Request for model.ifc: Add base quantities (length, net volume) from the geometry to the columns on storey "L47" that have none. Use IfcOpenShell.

First a look at what the model holds.

```python
import ifcopenshell
import ifcopenshell.util.element
import ifcopenshell.util.unit

model = ifcopenshell.open("model.ifc")
print(model.schema)
for unit_type in ("LENGTHUNIT", "AREAUNIT", "VOLUMEUNIT"):
    print(unit_type, ifcopenshell.util.unit.calculate_unit_scale(model, unit_type))
storey = next(s for s in model.by_type("IfcBuildingStorey") if s.Name == "L47")
columns = [e for e in ifcopenshell.util.element.get_decomposition(storey) if e.is_a("IfcColumn")]
for e in sorted(columns, key=lambda e: e.id()):
    print(e.id(), e.is_a(), e.Name, list(ifcopenshell.util.element.get_psets(e, qtos_only=True)), sep=" | ")
```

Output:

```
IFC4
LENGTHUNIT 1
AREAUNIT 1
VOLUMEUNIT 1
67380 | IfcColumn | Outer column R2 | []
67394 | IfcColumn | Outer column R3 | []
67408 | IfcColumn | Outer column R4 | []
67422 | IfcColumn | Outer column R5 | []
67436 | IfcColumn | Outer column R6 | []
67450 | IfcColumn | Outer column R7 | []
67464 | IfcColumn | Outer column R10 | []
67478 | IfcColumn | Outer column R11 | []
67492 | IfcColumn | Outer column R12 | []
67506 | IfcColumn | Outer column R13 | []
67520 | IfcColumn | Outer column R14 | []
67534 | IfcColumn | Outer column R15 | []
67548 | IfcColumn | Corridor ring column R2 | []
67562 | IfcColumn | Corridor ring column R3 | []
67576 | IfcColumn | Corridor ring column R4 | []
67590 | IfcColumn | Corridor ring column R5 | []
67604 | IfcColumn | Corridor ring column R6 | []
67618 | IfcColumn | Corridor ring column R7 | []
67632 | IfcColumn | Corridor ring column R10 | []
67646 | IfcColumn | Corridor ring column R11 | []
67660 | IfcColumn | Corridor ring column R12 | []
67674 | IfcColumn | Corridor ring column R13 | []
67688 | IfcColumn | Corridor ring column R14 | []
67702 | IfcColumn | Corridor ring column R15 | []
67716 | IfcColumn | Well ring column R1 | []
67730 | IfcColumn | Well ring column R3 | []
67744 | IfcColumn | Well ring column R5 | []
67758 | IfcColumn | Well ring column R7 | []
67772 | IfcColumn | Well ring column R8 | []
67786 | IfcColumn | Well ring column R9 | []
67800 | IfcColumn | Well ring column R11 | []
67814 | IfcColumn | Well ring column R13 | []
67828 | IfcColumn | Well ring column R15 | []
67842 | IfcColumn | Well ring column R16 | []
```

```python
import ifcopenshell
import ifcopenshell.api.pset
import ifcopenshell.geom
import ifcopenshell.util.element
import ifcopenshell.util.shape
import ifcopenshell.util.unit

model = ifcopenshell.open("model.ifc")
unit_scale = ifcopenshell.util.unit.calculate_unit_scale(model)
volume_scale = ifcopenshell.util.unit.calculate_unit_scale(model, "VOLUMEUNIT")
settings = ifcopenshell.geom.settings()

storey = next(s for s in model.by_type("IfcBuildingStorey") if s.Name == "L47")
columns = [e for e in ifcopenshell.util.element.get_decomposition(storey) if e.is_a("IfcColumn")]

for e in sorted(columns, key=lambda e: e.id()):
    if ifcopenshell.util.element.get_psets(e, qtos_only=True, should_inherit=False):
        continue
    # Geometry comes back in metres, in the element's own axes.
    shape = ifcopenshell.geom.create_shape(settings, e)
    values = {
        "Length": ifcopenshell.util.shape.get_z(shape.geometry) / unit_scale,
        "NetVolume": ifcopenshell.util.shape.get_volume(shape.geometry) / volume_scale,
    }
    qto = ifcopenshell.api.pset.add_qto(model, product=e, name="Qto_ColumnBaseQuantities")
    ifcopenshell.api.pset.edit_qto(model, qto=qto, properties=values)
    print(e.id(), {k: round(v, 3) for k, v in values.items()})

model.write("model_rev.ifc")
```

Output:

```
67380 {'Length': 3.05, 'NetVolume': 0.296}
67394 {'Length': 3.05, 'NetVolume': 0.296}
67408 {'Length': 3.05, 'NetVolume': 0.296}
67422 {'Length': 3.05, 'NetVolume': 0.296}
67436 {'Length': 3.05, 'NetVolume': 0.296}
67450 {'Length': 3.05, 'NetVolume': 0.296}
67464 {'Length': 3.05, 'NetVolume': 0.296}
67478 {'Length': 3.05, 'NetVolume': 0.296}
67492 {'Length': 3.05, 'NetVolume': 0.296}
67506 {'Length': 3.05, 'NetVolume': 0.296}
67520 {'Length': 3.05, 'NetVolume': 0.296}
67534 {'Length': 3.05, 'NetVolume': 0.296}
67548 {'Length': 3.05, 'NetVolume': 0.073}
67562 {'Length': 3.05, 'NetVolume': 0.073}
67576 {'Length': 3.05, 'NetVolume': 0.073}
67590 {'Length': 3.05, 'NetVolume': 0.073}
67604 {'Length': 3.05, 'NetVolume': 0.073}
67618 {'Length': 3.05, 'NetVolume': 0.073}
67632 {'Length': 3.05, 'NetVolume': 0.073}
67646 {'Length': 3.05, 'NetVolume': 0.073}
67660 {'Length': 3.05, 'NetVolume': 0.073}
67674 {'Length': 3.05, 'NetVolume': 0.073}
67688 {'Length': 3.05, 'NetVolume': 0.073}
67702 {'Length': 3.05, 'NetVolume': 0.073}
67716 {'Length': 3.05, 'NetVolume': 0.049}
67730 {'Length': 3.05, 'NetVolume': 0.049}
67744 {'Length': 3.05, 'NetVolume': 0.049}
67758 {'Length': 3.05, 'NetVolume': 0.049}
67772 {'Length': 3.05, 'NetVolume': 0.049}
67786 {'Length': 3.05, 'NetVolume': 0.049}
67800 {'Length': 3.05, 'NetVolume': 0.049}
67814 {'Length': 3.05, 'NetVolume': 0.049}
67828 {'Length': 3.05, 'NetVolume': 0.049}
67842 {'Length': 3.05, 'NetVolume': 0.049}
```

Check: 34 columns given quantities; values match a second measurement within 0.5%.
